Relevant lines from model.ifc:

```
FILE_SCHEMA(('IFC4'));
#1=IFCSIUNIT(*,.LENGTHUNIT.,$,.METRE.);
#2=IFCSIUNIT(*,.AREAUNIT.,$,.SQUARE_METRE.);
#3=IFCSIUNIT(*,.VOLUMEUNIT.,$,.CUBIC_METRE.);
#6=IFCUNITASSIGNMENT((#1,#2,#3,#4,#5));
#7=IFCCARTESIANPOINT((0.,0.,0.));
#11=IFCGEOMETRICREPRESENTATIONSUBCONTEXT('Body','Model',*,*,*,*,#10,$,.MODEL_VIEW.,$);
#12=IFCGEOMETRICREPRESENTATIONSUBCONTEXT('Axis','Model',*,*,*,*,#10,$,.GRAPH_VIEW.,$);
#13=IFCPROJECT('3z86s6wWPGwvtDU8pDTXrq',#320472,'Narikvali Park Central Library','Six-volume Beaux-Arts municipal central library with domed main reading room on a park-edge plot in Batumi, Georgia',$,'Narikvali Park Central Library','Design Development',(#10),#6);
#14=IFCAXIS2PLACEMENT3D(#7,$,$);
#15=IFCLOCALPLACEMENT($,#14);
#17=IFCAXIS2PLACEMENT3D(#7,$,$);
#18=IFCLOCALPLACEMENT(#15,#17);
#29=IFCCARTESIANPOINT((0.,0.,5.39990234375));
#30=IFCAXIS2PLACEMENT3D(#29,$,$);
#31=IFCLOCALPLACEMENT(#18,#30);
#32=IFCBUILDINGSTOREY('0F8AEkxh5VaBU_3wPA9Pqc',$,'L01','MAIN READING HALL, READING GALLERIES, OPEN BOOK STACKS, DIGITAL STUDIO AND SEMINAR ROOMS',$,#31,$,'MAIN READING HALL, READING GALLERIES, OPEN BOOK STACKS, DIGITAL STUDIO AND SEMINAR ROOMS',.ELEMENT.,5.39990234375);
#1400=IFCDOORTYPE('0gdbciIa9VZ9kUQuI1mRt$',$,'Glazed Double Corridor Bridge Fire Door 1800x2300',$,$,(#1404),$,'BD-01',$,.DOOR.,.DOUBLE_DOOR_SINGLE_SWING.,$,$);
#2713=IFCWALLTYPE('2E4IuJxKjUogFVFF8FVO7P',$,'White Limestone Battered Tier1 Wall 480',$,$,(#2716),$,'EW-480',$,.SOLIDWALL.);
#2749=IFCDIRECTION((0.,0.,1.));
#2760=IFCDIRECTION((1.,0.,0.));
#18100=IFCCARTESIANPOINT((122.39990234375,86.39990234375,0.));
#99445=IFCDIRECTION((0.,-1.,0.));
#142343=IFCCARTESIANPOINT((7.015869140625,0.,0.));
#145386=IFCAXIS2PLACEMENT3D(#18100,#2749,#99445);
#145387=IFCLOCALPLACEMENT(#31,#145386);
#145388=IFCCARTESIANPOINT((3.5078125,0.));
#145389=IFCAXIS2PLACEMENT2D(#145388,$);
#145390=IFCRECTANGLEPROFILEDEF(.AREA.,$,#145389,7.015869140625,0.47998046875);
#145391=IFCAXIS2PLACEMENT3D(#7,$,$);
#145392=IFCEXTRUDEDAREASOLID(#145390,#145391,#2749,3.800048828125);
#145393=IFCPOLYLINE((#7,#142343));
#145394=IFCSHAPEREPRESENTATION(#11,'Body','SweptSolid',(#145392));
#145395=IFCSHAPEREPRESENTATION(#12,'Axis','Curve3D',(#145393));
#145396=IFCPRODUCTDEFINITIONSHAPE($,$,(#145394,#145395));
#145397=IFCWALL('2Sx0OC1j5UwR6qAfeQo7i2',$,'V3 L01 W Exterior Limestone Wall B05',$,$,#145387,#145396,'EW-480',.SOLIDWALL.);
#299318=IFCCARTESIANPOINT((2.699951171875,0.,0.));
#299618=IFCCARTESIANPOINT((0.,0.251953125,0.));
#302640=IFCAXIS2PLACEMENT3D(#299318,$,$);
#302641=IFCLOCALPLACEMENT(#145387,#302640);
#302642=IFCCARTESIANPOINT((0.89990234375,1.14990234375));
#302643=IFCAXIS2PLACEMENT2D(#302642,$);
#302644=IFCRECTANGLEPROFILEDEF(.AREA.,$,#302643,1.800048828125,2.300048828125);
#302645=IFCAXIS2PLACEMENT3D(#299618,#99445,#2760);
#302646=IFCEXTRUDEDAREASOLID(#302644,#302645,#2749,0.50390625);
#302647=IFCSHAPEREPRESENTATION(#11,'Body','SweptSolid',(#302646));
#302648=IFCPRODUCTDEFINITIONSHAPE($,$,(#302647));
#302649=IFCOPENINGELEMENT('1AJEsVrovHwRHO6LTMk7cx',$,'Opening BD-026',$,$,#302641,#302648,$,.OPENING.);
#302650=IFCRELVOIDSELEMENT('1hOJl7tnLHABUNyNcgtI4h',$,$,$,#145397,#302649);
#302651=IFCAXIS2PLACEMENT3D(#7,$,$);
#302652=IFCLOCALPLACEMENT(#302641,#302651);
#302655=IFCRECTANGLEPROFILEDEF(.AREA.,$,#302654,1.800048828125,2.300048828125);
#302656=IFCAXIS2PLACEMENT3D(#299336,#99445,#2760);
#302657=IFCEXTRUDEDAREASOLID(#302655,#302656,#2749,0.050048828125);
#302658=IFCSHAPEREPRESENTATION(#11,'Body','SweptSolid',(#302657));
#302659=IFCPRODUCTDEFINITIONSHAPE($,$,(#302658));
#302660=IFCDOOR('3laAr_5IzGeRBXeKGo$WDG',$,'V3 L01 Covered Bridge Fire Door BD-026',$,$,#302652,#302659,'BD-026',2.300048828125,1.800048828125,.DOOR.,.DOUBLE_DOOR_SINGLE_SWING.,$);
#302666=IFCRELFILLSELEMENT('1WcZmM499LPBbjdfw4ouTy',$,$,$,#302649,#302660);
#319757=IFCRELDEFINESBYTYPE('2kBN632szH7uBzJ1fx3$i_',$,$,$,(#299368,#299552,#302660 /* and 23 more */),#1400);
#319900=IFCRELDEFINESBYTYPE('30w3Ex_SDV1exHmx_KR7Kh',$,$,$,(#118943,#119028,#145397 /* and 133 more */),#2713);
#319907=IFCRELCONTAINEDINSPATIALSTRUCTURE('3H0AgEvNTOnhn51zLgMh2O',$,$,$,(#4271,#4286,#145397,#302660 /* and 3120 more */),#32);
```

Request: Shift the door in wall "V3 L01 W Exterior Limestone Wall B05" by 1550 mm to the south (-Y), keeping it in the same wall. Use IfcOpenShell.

```python
import ifcopenshell
import ifcopenshell.api.geometry
import ifcopenshell.util.placement

model = ifcopenshell.open("model.ifc")

door = model.by_guid("3laAr_5IzGeRBXeKGo$WDG")
opening = door.FillsVoids[0].RelatingOpeningElement
wall = opening.VoidsElements[0].RelatingBuildingElement

wall_matrix = ifcopenshell.util.placement.get_local_placement(wall.ObjectPlacement)
shift = wall_matrix[:3, 0] * 1.55
before = ifcopenshell.util.placement.get_local_placement(door.ObjectPlacement)[:3, 3].copy()

# The door is placed relative to its opening, so it follows when the opening moves.
matrix = ifcopenshell.util.placement.get_local_placement(opening.ObjectPlacement)
matrix[:3, 3] += shift
ifcopenshell.api.geometry.edit_object_placement(
    model, product=opening, matrix=matrix, is_si=False, should_transform_children=True
)

after = ifcopenshell.util.placement.get_local_placement(door.ObjectPlacement)[:3, 3]
print("door moved by", (after - before).round(3) + 0.0)

model.write("model_edited.ifc")
```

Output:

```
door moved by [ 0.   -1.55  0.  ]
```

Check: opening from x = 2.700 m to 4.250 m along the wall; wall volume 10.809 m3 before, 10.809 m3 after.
